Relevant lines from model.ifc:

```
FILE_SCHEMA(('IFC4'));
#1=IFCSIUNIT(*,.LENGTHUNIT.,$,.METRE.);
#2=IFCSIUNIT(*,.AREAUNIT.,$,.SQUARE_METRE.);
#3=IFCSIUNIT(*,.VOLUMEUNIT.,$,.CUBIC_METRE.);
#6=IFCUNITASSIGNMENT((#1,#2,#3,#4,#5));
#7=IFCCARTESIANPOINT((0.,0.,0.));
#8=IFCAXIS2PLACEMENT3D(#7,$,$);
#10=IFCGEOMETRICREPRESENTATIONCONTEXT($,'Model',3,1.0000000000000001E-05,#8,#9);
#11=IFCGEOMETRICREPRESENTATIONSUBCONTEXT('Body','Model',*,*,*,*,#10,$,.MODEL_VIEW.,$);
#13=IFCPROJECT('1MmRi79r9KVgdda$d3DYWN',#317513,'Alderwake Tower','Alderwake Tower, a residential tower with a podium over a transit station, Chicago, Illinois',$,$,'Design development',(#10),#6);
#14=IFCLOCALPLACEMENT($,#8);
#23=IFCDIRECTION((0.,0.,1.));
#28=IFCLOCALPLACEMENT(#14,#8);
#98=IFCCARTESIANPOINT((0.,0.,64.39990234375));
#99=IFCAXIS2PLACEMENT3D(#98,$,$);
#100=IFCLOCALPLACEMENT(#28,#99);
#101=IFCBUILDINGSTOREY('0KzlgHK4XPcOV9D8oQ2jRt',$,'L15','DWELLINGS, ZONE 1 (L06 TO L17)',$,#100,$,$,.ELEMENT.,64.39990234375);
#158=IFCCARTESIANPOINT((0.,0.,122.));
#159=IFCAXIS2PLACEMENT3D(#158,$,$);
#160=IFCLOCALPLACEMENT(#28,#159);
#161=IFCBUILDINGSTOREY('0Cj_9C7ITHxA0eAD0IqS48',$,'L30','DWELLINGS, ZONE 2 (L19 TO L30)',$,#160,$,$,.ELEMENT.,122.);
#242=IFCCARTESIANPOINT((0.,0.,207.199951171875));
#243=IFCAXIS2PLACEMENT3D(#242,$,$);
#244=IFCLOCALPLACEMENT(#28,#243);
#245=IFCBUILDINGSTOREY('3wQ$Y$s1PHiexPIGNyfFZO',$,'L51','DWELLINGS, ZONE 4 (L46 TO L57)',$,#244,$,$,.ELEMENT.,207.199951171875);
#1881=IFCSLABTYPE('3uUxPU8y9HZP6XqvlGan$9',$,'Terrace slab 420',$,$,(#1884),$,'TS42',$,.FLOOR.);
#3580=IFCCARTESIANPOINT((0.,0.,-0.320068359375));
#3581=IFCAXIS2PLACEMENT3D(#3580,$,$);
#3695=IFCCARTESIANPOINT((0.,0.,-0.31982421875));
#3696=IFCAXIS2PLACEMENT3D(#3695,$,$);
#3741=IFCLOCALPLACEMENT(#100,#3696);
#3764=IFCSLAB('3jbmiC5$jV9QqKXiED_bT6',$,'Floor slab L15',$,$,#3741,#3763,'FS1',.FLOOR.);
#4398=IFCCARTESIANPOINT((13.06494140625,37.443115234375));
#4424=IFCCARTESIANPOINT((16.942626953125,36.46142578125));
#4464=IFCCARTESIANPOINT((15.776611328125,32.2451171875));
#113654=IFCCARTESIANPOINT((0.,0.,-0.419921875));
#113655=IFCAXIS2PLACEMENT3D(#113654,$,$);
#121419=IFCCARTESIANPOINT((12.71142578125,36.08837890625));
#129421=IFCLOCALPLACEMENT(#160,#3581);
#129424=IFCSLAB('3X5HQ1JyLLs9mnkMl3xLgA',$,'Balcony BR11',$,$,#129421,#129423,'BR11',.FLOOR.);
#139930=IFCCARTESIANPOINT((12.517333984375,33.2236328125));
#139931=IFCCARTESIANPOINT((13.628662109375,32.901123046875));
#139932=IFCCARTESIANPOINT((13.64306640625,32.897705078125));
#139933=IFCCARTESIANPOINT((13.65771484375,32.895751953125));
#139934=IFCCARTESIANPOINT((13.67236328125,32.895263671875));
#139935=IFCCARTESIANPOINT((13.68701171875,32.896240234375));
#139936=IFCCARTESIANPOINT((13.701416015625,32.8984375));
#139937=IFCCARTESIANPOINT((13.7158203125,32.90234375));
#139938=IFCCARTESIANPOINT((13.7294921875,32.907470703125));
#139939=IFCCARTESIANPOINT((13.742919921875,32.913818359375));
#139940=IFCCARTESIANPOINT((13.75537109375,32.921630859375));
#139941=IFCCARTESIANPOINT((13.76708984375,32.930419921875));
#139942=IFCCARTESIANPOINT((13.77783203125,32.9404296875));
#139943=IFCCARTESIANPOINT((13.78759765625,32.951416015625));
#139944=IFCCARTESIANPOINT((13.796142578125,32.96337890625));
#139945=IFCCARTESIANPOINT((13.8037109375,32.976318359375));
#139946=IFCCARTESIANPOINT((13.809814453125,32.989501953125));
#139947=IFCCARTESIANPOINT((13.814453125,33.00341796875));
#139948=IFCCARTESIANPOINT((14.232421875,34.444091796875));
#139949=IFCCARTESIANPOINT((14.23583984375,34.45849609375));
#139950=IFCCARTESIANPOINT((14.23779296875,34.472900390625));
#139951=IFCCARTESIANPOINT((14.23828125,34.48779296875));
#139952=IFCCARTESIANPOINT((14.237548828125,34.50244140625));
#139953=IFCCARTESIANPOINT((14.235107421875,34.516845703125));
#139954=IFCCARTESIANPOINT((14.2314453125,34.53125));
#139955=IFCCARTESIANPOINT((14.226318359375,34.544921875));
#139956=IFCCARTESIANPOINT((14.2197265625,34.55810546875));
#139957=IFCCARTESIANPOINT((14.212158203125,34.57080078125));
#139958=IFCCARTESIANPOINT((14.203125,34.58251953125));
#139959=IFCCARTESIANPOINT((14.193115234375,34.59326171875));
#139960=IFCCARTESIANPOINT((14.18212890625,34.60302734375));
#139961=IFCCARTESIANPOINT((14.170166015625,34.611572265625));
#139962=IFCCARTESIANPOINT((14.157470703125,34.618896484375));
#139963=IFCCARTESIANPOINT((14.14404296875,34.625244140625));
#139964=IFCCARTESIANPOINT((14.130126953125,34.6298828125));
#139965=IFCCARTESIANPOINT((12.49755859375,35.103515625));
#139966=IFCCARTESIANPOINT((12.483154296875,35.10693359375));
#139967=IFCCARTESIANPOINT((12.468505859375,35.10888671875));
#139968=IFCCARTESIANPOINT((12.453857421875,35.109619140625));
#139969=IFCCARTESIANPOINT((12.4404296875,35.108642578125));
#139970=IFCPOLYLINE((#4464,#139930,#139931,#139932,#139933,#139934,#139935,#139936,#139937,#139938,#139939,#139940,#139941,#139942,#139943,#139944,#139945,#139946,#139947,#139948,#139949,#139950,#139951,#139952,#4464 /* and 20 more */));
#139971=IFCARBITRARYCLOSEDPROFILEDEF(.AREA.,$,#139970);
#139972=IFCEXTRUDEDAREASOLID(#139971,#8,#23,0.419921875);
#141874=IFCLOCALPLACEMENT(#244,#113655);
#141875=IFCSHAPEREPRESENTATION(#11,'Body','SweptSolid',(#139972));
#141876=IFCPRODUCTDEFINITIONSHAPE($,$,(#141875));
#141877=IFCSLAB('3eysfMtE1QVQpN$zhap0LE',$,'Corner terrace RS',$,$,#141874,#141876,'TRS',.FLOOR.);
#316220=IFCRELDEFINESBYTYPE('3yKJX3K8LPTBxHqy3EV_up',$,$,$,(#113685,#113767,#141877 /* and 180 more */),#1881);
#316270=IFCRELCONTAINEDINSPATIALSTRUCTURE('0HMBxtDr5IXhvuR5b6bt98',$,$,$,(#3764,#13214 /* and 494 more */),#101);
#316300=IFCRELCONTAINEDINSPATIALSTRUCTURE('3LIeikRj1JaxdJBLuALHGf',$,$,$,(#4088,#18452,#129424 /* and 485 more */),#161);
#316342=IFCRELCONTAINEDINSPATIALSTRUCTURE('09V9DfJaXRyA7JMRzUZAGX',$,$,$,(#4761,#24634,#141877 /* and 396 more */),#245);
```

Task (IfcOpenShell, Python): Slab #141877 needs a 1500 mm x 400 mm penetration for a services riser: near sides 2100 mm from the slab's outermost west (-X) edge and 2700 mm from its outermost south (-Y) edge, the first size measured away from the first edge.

```python
import numpy as np
import ifcopenshell
import ifcopenshell.api.feature
import ifcopenshell.api.geometry
import ifcopenshell.api.root
import ifcopenshell.geom
import ifcopenshell.util.placement
import ifcopenshell.util.representation
import ifcopenshell.util.shape
import ifcopenshell.util.unit

model = ifcopenshell.open("model.ifc")
unit_scale = ifcopenshell.util.unit.calculate_unit_scale(model)
settings = ifcopenshell.geom.settings()


def volume(element):
    """Net volume in cubic metres, openings subtracted."""
    shape = ifcopenshell.geom.create_shape(settings, element)
    return ifcopenshell.util.shape.get_volume(shape.geometry)


slab = model.by_guid("3eysfMtE1QVQpN$zhap0LE")
before = volume(slab)

# Extent in the slab's own axes, in metres. The edges named are its -X and -Y sides.
slab_shape = ifcopenshell.geom.create_shape(settings, slab)
vertices = ifcopenshell.util.shape.get_vertices(slab_shape.geometry)
x_min, y_min, bottom = vertices.min(axis=0)
top = vertices[:, 2].max()

opening = ifcopenshell.api.root.create_entity(model, ifc_class="IfcOpeningElement", name="Services riser opening", predefined_type="OPENING")
context = ifcopenshell.util.representation.get_context(model, "Model", "Body", "MODEL_VIEW")
width, depth = 1.5, 0.4
outline = [(0.0, 0.0), (width, 0.0), (width, depth), (0.0, depth), (0.0, 0.0)]
# Overshoot both faces by 50 mm so the cut is clean.
shape = ifcopenshell.api.geometry.add_slab_representation(
    model, context=context, depth=top - bottom + 0.1, polyline=outline
)
ifcopenshell.api.geometry.assign_representation(model, product=opening, representation=shape)

matrix = ifcopenshell.util.placement.get_local_placement(slab.ObjectPlacement)
matrix[:, 3] = matrix @ np.append(np.array([x_min + 2.1, y_min + 2.7, bottom - 0.05]) / unit_scale, 1.0)
ifcopenshell.api.geometry.edit_object_placement(model, product=opening, matrix=matrix, is_si=False)
ifcopenshell.api.feature.add_feature(model, feature=opening, element=slab)

after = volume(slab)

print(f"slab volume {before:.3f} -> {after:.3f} m3")

model.write("model_v2.ifc")
```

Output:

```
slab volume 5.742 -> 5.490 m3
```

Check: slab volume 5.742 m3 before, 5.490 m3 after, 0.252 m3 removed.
